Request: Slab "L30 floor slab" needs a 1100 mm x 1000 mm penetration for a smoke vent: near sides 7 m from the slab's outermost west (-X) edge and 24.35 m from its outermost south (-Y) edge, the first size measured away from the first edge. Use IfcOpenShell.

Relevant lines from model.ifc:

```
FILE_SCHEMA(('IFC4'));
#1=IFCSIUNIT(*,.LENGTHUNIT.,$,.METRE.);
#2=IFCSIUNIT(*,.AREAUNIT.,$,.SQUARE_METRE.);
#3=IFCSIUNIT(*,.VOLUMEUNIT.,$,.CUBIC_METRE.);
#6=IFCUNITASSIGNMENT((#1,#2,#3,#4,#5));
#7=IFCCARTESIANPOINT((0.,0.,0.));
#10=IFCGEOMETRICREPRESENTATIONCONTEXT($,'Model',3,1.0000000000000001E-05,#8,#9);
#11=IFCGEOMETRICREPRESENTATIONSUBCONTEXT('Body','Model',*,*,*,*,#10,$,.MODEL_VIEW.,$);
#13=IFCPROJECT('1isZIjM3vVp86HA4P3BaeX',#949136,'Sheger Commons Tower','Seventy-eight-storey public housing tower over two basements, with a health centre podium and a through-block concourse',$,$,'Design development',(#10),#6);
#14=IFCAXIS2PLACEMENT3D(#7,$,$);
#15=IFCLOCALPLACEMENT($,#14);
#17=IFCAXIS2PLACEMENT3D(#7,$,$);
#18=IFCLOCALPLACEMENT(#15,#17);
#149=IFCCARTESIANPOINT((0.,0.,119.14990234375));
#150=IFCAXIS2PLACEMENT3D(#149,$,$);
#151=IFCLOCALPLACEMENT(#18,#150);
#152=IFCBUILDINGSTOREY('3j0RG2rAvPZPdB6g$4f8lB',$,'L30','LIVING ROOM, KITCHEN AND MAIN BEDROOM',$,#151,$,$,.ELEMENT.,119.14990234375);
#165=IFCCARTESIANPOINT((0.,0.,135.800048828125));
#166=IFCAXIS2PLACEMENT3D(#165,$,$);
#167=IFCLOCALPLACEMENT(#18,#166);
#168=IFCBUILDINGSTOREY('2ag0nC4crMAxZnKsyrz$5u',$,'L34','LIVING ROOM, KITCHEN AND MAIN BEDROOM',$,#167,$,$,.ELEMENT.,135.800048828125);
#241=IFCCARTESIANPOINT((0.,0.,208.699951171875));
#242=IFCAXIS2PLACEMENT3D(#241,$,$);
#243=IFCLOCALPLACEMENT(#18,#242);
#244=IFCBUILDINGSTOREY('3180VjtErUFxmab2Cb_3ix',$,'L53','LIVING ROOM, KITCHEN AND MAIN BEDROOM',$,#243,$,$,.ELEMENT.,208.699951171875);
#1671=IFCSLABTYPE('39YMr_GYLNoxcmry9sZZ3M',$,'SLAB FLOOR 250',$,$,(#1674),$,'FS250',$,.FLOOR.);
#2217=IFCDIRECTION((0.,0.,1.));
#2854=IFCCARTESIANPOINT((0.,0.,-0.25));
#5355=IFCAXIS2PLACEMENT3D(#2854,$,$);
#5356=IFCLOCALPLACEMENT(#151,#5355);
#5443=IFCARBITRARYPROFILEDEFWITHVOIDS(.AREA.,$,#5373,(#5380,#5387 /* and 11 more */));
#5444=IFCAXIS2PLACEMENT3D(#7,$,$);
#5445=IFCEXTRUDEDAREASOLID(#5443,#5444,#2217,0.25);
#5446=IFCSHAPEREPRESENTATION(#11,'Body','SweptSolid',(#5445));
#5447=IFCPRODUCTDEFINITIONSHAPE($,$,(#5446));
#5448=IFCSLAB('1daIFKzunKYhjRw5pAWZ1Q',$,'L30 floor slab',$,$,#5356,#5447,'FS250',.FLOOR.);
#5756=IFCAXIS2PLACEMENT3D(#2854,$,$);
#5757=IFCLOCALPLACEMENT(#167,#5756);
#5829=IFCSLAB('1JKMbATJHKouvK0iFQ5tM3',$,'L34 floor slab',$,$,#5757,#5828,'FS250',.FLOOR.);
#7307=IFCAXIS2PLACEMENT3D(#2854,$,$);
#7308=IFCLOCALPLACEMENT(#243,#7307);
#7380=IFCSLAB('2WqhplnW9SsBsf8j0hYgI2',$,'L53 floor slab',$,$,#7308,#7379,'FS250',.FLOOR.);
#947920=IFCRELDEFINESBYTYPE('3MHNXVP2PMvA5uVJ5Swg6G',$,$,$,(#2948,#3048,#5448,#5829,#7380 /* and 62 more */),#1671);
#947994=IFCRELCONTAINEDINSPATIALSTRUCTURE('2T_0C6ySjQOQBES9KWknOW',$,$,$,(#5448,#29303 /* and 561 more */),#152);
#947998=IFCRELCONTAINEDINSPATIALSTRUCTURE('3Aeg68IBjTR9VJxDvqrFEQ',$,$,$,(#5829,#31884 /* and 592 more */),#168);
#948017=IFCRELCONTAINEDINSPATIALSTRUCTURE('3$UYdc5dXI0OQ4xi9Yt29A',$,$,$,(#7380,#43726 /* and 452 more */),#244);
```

```python
import numpy as np
import ifcopenshell
import ifcopenshell.api.feature
import ifcopenshell.api.geometry
import ifcopenshell.api.root
import ifcopenshell.geom
import ifcopenshell.util.placement
import ifcopenshell.util.representation
import ifcopenshell.util.shape
import ifcopenshell.util.unit

model = ifcopenshell.open("model.ifc")
unit_scale = ifcopenshell.util.unit.calculate_unit_scale(model)
settings = ifcopenshell.geom.settings()


def volume(element):
    """Net volume in cubic metres, openings subtracted."""
    shape = ifcopenshell.geom.create_shape(settings, element)
    return ifcopenshell.util.shape.get_volume(shape.geometry)


slab = model.by_guid("1daIFKzunKYhjRw5pAWZ1Q")
before = volume(slab)

# Extent in the slab's own axes, in metres. The edges named are its -X and -Y sides.
slab_shape = ifcopenshell.geom.create_shape(settings, slab)
vertices = ifcopenshell.util.shape.get_vertices(slab_shape.geometry)
x_min, y_min, bottom = vertices.min(axis=0)
top = vertices[:, 2].max()

opening = ifcopenshell.api.root.create_entity(model, ifc_class="IfcOpeningElement", name="Smoke vent opening", predefined_type="OPENING")
context = ifcopenshell.util.representation.get_context(model, "Model", "Body", "MODEL_VIEW")
width, depth = 1.1, 1
outline = [(0.0, 0.0), (width, 0.0), (width, depth), (0.0, depth), (0.0, 0.0)]
# Overshoot both faces by 50 mm so the cut is clean.
shape = ifcopenshell.api.geometry.add_slab_representation(
    model, context=context, depth=top - bottom + 0.1, polyline=outline
)
ifcopenshell.api.geometry.assign_representation(model, product=opening, representation=shape)

matrix = ifcopenshell.util.placement.get_local_placement(slab.ObjectPlacement)
matrix[:, 3] = matrix @ np.append(np.array([x_min + 7, y_min + 24.35, bottom - 0.05]) / unit_scale, 1.0)
ifcopenshell.api.geometry.edit_object_placement(model, product=opening, matrix=matrix, is_si=False)
ifcopenshell.api.feature.add_feature(model, feature=opening, element=slab)

after = volume(slab)

print(f"slab volume {before:.3f} -> {after:.3f} m3")

model.write("model_updated.ifc")
```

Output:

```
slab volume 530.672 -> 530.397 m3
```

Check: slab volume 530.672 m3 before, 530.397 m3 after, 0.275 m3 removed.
